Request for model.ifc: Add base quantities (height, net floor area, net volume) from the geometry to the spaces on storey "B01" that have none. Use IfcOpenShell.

First a look at what the model holds.

```python
import ifcopenshell
import ifcopenshell.util.element
import ifcopenshell.util.unit

model = ifcopenshell.open("model.ifc")
print(model.schema)
for unit_type in ("LENGTHUNIT", "AREAUNIT", "VOLUMEUNIT"):
    print(unit_type, ifcopenshell.util.unit.calculate_unit_scale(model, unit_type))
storey = next(s for s in model.by_type("IfcBuildingStorey") if s.Name == "B01")
spaces = [e for e in ifcopenshell.util.element.get_decomposition(storey) if e.is_a("IfcSpace")]
for e in sorted(spaces, key=lambda e: e.id()):
    print(e.id(), e.is_a(), e.Name, list(ifcopenshell.util.element.get_psets(e, qtos_only=True)), sep=" | ")
```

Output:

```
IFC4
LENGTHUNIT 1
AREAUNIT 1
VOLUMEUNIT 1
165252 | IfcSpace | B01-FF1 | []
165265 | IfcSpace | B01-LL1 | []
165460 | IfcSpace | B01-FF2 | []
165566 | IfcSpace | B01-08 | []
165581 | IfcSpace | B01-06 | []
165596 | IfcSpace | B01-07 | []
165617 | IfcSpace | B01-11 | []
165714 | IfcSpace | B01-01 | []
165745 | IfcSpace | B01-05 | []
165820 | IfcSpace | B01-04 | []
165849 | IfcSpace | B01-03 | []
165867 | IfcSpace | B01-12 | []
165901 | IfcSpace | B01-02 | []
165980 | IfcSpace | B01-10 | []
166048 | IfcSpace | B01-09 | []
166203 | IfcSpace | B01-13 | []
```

```python
import ifcopenshell
import ifcopenshell.api.pset
import ifcopenshell.geom
import ifcopenshell.util.element
import ifcopenshell.util.shape
import ifcopenshell.util.unit

model = ifcopenshell.open("model.ifc")
unit_scale = ifcopenshell.util.unit.calculate_unit_scale(model)
area_scale = ifcopenshell.util.unit.calculate_unit_scale(model, "AREAUNIT")
volume_scale = ifcopenshell.util.unit.calculate_unit_scale(model, "VOLUMEUNIT")
settings = ifcopenshell.geom.settings()

storey = next(s for s in model.by_type("IfcBuildingStorey") if s.Name == "B01")
spaces = [e for e in ifcopenshell.util.element.get_decomposition(storey) if e.is_a("IfcSpace")]

for e in sorted(spaces, key=lambda e: e.id()):
    if ifcopenshell.util.element.get_psets(e, qtos_only=True, should_inherit=False):
        continue
    # Geometry comes back in metres, in the element's own axes.
    shape = ifcopenshell.geom.create_shape(settings, e)
    values = {
        "Height": ifcopenshell.util.shape.get_z(shape.geometry) / unit_scale,
        "NetFloorArea": ifcopenshell.util.shape.get_footprint_area(shape.geometry) / area_scale,
        "NetVolume": ifcopenshell.util.shape.get_volume(shape.geometry) / volume_scale,
    }
    qto = ifcopenshell.api.pset.add_qto(model, product=e, name="Qto_SpaceBaseQuantities")
    ifcopenshell.api.pset.edit_qto(model, qto=qto, properties=values)
    print(e.id(), {k: round(v, 3) for k, v in values.items()})

model.write("model-out.ifc")
```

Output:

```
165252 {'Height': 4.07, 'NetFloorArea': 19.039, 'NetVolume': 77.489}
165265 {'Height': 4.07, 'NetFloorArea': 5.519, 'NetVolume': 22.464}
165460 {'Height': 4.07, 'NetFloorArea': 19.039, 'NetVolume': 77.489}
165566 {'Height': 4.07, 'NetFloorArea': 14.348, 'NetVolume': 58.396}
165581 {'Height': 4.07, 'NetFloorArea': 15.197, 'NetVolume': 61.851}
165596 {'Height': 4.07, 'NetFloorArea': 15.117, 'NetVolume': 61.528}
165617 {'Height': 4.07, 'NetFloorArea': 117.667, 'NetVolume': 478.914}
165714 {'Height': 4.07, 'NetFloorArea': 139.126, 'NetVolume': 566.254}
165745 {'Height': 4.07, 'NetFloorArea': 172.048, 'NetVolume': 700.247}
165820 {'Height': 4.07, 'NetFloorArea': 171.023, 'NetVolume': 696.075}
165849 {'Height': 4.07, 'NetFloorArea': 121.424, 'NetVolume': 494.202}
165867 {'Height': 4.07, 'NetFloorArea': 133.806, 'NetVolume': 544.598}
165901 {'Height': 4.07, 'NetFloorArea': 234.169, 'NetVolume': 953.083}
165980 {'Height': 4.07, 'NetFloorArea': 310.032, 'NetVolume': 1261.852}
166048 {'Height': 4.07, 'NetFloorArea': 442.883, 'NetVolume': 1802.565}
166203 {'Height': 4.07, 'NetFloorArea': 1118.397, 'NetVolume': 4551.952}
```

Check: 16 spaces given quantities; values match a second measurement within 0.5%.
